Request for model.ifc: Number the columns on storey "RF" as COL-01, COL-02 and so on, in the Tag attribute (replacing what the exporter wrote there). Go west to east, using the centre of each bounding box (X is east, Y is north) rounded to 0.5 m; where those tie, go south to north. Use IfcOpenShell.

First a look at what the model holds.

```python
import ifcopenshell
import ifcopenshell.util.element
import ifcopenshell.util.placement

model = ifcopenshell.open("model.ifc")
print(model.schema)
storey = next(s for s in model.by_type("IfcBuildingStorey") if s.Name == "RF")
columns = [e for e in ifcopenshell.util.element.get_decomposition(storey) if e.is_a("IfcColumn")]
for e in sorted(columns, key=lambda e: e.id()):
    origin = ifcopenshell.util.placement.get_local_placement(e.ObjectPlacement)[:3, 3]
    print(e.id(), e.Tag, e.Name, origin.round(2) + 0.0, sep=" | ")
```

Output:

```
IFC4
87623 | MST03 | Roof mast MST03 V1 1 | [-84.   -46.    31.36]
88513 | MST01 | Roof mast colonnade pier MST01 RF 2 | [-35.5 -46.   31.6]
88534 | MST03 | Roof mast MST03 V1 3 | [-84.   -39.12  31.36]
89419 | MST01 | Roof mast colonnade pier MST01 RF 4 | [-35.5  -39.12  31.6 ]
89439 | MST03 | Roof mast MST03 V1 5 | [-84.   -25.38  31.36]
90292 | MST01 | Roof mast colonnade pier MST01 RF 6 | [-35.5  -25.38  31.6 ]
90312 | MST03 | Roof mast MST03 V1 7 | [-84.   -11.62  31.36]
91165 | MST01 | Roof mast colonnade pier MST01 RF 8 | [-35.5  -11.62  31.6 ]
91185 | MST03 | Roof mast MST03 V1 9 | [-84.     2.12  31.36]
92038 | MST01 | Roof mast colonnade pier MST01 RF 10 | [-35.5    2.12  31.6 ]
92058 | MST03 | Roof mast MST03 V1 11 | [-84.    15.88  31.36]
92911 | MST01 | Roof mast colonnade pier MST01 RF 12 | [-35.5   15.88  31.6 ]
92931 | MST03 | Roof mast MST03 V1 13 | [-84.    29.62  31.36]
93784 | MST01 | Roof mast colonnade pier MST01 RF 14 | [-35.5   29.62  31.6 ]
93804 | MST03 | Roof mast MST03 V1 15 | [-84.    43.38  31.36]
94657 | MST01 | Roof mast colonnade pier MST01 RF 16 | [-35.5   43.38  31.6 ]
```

```python
import ifcopenshell
import ifcopenshell.geom
import ifcopenshell.util.element
import ifcopenshell.util.shape

model = ifcopenshell.open("model.ifc")
settings = ifcopenshell.geom.settings()
settings.set("use-world-coords", True)


def centre(element):
    shape = ifcopenshell.geom.create_shape(settings, element)
    return ifcopenshell.util.shape.get_bbox_centroid(shape.geometry)


storey = next(s for s in model.by_type("IfcBuildingStorey") if s.Name == "RF")
columns = [e for e in ifcopenshell.util.element.get_decomposition(storey) if e.is_a("IfcColumn")]

# Insertion points can sit at a corner or the storey origin, so sort by the geometry (in metres).
centres = {e: centre(e) for e in columns}
columns.sort(key=lambda e: (round(centres[e][0] / 0.5), centres[e][1]))

for i, e in enumerate(columns, start=1):
    number = f"COL-{i:02d}"
    e.Tag = number
    print(e.id(), number)

model.write("model_updated.ifc")
```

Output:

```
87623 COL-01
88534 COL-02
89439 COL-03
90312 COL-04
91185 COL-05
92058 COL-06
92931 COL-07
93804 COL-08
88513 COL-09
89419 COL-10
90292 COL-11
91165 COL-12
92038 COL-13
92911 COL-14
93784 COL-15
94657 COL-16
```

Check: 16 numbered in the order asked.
